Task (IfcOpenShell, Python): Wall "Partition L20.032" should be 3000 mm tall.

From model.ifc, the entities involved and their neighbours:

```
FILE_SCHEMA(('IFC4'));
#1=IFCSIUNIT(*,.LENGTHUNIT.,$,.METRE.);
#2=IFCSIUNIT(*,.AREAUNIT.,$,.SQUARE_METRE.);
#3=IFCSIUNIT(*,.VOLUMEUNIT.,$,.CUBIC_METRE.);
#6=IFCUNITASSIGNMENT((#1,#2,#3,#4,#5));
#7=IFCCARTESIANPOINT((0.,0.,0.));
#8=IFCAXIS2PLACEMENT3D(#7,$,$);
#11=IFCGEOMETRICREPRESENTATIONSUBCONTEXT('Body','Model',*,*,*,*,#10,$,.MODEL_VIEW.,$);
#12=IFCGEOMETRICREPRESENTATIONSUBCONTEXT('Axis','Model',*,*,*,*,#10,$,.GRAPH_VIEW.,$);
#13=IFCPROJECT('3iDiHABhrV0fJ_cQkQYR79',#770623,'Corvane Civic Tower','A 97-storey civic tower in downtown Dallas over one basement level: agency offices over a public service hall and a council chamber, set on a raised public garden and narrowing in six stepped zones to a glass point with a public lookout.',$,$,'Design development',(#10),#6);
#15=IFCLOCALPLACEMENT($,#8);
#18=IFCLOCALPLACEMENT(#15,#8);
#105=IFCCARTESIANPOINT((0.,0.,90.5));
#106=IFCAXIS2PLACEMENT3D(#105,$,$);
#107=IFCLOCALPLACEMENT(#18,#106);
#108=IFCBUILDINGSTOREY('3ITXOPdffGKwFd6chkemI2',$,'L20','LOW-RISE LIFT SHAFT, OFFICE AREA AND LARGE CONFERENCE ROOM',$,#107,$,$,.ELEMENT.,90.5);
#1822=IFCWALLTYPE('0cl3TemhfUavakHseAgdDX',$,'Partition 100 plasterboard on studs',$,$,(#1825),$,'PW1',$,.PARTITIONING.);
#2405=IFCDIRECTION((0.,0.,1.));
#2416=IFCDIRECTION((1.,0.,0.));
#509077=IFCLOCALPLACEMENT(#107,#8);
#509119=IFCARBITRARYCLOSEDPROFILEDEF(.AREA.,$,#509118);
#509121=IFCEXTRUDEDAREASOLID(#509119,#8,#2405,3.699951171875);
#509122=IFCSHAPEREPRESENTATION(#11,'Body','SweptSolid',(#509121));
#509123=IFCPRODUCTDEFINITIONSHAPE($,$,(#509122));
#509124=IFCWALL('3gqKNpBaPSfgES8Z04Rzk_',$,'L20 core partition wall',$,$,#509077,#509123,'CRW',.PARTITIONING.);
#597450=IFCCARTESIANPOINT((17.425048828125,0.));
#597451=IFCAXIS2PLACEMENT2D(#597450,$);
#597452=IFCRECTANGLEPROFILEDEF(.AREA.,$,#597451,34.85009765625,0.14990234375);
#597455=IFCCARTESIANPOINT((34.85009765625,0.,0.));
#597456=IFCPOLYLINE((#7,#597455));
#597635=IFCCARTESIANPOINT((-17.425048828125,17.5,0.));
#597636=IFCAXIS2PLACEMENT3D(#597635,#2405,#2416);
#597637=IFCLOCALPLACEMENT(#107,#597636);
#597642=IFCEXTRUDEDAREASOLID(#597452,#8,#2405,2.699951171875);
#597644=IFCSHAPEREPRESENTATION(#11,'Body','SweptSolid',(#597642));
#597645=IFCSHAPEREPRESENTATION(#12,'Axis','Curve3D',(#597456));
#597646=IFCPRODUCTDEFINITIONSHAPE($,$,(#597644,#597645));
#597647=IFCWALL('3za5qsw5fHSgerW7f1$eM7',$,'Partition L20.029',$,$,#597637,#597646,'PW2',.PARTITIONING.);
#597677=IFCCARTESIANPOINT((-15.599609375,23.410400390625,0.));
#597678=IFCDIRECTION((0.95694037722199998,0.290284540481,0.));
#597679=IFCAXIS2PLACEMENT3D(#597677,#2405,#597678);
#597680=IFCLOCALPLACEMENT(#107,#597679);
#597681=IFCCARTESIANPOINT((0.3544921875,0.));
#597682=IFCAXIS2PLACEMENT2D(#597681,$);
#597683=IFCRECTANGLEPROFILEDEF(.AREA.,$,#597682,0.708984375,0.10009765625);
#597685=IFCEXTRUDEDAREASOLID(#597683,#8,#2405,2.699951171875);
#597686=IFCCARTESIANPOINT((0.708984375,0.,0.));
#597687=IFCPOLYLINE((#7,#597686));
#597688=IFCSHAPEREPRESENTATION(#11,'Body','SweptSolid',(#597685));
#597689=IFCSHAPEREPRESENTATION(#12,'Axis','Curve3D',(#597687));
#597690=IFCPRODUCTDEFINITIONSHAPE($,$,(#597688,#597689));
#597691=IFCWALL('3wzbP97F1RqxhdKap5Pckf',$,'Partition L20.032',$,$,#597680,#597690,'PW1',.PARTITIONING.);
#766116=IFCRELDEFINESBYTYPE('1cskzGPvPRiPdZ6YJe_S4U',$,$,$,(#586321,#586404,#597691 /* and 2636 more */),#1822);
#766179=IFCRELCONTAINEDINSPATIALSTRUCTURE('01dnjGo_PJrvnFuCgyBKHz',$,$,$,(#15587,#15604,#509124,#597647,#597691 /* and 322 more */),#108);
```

```python
import ifcopenshell
import ifcopenshell.geom
import ifcopenshell.util.representation
import ifcopenshell.util.shape

model = ifcopenshell.open("model.ifc")
settings = ifcopenshell.geom.settings()


def volume(element):
    """Net volume in cubic metres, openings subtracted."""
    shape = ifcopenshell.geom.create_shape(settings, element)
    return ifcopenshell.util.shape.get_volume(shape.geometry)


wall = model.by_id(597691)
before = volume(wall)

body = ifcopenshell.util.representation.get_representation(wall, "Model", "Body")
solid = body.Items[0]
old_height = solid.Depth
solid.Depth = 3.0
after = volume(wall)

print(f"height {old_height:g} -> {solid.Depth:g}, volume {before:.3f} -> {after:.3f} m3")

model.write("model-out.ifc")
```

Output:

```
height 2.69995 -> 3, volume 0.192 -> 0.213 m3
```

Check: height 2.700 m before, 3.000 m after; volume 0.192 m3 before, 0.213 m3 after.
